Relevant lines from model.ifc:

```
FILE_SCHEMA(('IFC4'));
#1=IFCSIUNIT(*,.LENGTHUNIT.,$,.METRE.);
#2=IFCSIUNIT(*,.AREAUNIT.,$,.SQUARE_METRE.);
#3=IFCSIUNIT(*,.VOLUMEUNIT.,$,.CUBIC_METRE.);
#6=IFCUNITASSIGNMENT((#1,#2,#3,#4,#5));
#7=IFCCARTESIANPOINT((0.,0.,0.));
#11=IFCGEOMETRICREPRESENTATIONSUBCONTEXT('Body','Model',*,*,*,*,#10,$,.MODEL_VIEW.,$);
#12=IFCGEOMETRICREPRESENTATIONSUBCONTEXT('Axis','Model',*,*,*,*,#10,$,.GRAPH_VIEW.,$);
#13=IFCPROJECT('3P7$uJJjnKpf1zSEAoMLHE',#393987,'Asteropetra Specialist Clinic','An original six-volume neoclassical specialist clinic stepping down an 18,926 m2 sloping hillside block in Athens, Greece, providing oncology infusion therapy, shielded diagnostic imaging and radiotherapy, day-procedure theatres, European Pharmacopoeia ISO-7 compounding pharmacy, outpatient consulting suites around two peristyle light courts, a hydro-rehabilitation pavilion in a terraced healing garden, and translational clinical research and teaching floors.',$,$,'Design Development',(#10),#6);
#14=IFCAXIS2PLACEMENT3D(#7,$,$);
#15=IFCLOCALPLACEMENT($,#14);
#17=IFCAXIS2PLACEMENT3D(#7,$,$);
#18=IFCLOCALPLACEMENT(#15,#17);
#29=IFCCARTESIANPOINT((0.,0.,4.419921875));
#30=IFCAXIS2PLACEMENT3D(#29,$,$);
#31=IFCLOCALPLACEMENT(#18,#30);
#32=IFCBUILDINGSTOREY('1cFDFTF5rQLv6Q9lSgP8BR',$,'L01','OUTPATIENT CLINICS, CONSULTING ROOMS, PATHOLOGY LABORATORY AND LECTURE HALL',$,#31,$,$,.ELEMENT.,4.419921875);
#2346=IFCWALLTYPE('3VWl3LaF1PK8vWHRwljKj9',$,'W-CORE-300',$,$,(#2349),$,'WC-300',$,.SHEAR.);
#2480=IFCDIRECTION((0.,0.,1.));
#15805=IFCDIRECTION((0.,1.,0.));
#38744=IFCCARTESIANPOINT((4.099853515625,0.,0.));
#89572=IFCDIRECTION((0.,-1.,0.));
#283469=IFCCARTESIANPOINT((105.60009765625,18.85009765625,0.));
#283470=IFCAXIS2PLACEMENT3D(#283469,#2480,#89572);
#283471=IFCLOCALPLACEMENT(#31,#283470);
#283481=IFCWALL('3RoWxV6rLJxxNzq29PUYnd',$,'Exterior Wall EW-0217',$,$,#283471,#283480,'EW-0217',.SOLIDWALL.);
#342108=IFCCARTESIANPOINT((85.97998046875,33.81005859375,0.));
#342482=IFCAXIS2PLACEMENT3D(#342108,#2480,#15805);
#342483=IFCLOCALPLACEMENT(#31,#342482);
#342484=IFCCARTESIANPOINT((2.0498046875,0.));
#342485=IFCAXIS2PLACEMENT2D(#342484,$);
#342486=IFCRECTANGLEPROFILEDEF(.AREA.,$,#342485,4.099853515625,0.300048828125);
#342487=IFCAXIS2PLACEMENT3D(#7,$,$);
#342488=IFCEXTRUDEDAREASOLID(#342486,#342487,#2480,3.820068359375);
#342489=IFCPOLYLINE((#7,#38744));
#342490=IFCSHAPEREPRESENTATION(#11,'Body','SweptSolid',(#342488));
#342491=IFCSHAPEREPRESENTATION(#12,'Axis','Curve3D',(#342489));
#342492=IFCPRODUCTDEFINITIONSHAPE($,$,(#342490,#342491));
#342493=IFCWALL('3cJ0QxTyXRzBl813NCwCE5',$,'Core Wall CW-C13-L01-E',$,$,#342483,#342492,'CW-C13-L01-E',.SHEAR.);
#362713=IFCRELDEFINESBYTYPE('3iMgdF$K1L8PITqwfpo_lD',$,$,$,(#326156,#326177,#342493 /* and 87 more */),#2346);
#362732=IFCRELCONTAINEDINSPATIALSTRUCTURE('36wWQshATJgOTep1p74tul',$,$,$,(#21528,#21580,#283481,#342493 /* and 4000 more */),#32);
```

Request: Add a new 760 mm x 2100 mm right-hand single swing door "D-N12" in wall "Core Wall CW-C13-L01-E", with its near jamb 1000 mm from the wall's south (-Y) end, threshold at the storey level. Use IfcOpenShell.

```python
import numpy as np
import ifcopenshell
import ifcopenshell.api.feature
import ifcopenshell.api.geometry
import ifcopenshell.api.root
import ifcopenshell.api.spatial
import ifcopenshell.geom
import ifcopenshell.util.element
import ifcopenshell.util.placement
import ifcopenshell.util.representation
import ifcopenshell.util.shape
import ifcopenshell.util.unit

model = ifcopenshell.open("model.ifc")
unit_scale = ifcopenshell.util.unit.calculate_unit_scale(model)
settings = ifcopenshell.geom.settings()


def volume(element):
    """Net volume in cubic metres, openings subtracted."""
    shape = ifcopenshell.geom.create_shape(settings, element)
    return ifcopenshell.util.shape.get_volume(shape.geometry)


wall = model.by_guid("3cJ0QxTyXRzBl813NCwCE5")
storey = ifcopenshell.util.element.get_container(wall, ifc_class="IfcBuildingStorey")
context = ifcopenshell.util.representation.get_context(model, "Model", "Body", "MODEL_VIEW")
before = volume(wall)

width, height, from_end, sill = 0.76, 2.1, 1, 0.0  # metres

# The wall runs along its own X axis, and the end named is its -X end.
wall_shape = ifcopenshell.geom.create_shape(settings, wall)
x, y, z = ifcopenshell.util.shape.get_vertices(wall_shape.geometry).T
start = x.min() + from_end
face, thickness = float(y.min()), float(y.max() - y.min())
wall_matrix = ifcopenshell.util.placement.get_local_placement(wall.ObjectPlacement)
level = ifcopenshell.util.placement.get_local_placement(storey.ObjectPlacement)[2, 3]


def in_wall(x, y):
    """Placement at x, y metres in the wall's axes, at sill height."""
    matrix = wall_matrix.copy()
    matrix[:, 3] = wall_matrix @ np.array([x / unit_scale, y / unit_scale, 0.0, 1.0])
    matrix[2, 3] = level + sill / unit_scale
    return matrix


# Opening: a box that overshoots both wall faces by 50 mm.
opening = ifcopenshell.api.root.create_entity(model, ifc_class="IfcOpeningElement", predefined_type="OPENING")
box = ifcopenshell.api.geometry.add_wall_representation(
    model, context=context, length=width, height=height, thickness=thickness + 0.1
)
ifcopenshell.api.geometry.assign_representation(model, product=opening, representation=box)
ifcopenshell.api.geometry.edit_object_placement(model, product=opening, matrix=in_wall(start, face - 0.05), is_si=False)
ifcopenshell.api.feature.add_feature(model, feature=opening, element=wall)

door = ifcopenshell.api.root.create_entity(model, ifc_class="IfcDoor", name="D-N12", predefined_type="DOOR")
door.OverallWidth, door.OverallHeight = width / unit_scale, height / unit_scale
door.OperationType = "SINGLE_SWING_RIGHT"
body = ifcopenshell.api.geometry.add_door_representation(
    model,
    context=context,
    overall_width=door.OverallWidth,
    overall_height=door.OverallHeight,
    operation_type="SINGLE_SWING_RIGHT",
    lining_properties={"LiningDepth": thickness / unit_scale, "ThresholdDepth": thickness / unit_scale},
)
ifcopenshell.api.geometry.assign_representation(model, product=door, representation=body)
ifcopenshell.api.spatial.assign_container(model, products=[door], relating_structure=storey)
ifcopenshell.api.feature.add_filling(model, opening=opening, element=door)

# The lining spans the wall, so the door starts at the wall face.
ifcopenshell.api.geometry.edit_object_placement(model, product=door, matrix=in_wall(start, face), is_si=False)

after = volume(wall)

print(f"wall volume {before:.3f} -> {after:.3f} m3")

model.write("model_rev.ifc")
```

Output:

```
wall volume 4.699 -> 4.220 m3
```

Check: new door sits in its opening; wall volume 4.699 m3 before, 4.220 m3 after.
